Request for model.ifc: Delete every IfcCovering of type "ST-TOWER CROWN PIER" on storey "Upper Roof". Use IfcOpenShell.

First a look at what the model holds.

```python
import ifcopenshell
import ifcopenshell.util.element

model = ifcopenshell.open("model.ifc")
print(model.schema)
storey = next(s for s in model.by_type("IfcBuildingStorey") if s.Name == "Upper Roof")
coverings = [e for e in ifcopenshell.util.element.get_decomposition(storey) if e.is_a("IfcCovering")]
seen = {}
for e in coverings:
    element_type = ifcopenshell.util.element.get_type(e)
    name = element_type.Name if element_type not in (None, e) else None
    seen[name] = seen.get(name, 0) + 1
for name, count in sorted(seen.items(), key=str):
    print(count, "x", name)
```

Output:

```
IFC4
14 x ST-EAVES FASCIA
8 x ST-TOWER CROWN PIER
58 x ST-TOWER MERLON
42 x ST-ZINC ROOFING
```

```python
import ifcopenshell
import ifcopenshell.api.root
import ifcopenshell.util.element

model = ifcopenshell.open("model.ifc")

storey = next(s for s in model.by_type("IfcBuildingStorey") if s.Name == "Upper Roof")
coverings = [e for e in ifcopenshell.util.element.get_decomposition(storey) if e.is_a("IfcCovering")]
targets = [e for e in coverings if (t := ifcopenshell.util.element.get_type(e)) not in (None, e) and t.Name == "ST-TOWER CROWN PIER"]

for e in targets:
    ifcopenshell.api.root.remove_product(model, product=e)
print(len(targets), "removed")

model.write("model_edited.ifc")
```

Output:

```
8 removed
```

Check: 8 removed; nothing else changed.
